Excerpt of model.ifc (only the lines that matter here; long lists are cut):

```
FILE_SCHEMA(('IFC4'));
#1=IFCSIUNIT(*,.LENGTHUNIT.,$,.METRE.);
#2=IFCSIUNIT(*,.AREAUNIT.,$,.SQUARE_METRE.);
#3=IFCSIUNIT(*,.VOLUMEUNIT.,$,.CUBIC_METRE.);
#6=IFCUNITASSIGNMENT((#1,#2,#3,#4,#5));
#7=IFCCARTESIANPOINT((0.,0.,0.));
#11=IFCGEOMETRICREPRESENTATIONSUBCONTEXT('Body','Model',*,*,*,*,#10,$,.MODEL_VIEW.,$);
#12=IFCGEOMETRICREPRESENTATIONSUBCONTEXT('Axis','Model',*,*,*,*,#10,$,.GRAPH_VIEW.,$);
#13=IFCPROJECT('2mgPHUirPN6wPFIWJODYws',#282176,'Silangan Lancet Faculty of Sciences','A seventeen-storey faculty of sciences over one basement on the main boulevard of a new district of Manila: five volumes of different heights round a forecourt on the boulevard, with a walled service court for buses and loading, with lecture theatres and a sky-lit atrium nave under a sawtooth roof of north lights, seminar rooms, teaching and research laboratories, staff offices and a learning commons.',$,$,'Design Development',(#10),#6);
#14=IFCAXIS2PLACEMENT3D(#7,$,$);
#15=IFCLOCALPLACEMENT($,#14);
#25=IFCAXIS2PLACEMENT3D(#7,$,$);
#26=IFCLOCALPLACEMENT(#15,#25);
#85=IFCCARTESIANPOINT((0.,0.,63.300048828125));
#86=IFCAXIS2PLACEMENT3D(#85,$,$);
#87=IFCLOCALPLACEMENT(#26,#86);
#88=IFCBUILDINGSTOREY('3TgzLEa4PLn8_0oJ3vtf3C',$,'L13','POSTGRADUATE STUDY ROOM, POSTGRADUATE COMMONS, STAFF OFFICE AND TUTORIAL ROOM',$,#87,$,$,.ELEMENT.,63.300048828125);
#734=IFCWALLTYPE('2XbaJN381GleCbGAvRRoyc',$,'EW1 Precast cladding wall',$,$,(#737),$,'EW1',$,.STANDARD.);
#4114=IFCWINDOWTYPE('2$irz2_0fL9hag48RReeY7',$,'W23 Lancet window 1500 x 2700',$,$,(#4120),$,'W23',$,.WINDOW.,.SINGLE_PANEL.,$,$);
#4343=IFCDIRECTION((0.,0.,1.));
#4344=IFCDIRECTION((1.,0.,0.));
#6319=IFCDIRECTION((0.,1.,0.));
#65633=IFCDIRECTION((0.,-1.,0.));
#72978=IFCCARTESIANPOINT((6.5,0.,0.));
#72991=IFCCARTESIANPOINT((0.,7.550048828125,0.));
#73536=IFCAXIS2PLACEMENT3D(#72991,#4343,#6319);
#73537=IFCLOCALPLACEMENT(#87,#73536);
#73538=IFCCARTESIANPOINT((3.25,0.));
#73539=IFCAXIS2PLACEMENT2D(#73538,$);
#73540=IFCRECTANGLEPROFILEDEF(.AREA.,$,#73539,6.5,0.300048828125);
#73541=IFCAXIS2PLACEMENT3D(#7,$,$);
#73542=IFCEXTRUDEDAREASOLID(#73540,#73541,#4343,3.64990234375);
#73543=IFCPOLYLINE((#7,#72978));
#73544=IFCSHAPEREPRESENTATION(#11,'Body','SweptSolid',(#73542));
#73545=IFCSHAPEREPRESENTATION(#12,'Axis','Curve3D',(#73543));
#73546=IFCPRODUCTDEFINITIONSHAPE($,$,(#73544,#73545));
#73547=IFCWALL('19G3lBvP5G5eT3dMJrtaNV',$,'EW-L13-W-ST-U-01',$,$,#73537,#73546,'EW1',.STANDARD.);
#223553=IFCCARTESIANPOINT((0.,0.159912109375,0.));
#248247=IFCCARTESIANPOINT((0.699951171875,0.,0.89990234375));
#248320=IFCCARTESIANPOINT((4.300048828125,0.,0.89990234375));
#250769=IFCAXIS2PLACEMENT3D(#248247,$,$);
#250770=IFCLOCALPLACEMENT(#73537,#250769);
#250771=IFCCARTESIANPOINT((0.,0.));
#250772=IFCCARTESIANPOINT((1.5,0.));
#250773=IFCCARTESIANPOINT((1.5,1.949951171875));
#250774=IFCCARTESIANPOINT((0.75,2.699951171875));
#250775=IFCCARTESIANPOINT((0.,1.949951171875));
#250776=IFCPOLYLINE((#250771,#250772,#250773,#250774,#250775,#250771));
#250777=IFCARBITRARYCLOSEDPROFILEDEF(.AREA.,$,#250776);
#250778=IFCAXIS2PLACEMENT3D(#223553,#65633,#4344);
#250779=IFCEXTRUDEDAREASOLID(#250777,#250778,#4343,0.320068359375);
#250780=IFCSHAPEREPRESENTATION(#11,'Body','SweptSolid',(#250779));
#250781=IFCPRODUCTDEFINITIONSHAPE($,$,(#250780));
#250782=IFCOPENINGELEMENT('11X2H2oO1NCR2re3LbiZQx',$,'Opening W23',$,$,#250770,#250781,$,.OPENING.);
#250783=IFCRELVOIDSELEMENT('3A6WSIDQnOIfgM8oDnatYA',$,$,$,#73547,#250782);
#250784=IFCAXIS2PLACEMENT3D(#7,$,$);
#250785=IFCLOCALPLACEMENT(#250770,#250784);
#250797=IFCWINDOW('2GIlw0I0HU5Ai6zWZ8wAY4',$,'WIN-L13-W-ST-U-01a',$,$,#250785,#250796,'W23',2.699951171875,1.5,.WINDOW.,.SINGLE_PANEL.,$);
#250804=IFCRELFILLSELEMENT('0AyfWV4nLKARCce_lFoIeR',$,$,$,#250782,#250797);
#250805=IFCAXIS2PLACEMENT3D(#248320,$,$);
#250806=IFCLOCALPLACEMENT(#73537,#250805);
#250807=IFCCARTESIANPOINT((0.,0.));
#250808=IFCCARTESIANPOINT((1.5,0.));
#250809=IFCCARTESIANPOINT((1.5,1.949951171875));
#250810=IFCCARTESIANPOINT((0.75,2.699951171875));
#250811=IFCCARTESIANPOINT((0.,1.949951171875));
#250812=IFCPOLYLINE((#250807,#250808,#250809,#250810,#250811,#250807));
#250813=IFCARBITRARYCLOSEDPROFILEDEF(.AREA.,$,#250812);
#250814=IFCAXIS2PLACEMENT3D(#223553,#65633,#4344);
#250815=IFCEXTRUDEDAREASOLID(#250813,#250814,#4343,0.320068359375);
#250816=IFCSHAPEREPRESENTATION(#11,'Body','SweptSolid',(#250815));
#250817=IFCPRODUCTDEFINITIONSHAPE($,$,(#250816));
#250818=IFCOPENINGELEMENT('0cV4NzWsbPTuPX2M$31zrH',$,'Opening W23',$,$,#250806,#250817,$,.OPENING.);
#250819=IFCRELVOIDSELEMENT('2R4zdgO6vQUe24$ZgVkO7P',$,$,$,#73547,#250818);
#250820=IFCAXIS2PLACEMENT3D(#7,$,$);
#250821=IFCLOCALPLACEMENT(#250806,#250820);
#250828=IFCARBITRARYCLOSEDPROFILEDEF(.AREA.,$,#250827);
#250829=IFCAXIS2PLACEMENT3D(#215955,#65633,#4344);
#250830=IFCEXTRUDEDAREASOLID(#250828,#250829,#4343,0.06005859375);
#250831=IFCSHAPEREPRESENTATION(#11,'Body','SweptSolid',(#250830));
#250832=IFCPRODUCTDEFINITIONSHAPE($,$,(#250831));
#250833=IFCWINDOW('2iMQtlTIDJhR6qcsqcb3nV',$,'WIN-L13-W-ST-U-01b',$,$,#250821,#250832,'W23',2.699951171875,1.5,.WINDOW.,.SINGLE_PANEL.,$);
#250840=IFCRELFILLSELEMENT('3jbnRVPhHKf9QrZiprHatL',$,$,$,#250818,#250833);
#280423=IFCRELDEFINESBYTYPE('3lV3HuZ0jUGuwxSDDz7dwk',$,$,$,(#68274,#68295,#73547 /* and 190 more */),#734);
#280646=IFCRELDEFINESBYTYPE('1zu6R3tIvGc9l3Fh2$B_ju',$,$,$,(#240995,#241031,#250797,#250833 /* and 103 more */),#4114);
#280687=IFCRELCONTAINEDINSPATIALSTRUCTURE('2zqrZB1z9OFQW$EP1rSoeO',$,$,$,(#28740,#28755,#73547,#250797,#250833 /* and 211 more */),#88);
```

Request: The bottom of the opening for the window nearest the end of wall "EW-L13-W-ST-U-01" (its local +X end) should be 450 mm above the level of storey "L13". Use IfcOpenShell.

```python
import numpy as np
import ifcopenshell
import ifcopenshell.api.geometry
import ifcopenshell.geom
import ifcopenshell.util.element
import ifcopenshell.util.placement
import ifcopenshell.util.shape
import ifcopenshell.util.unit

model = ifcopenshell.open("model.ifc")
unit_scale = ifcopenshell.util.unit.calculate_unit_scale(model)

window = model.by_id(250833)
opening = window.FillsVoids[0].RelatingOpeningElement
storey = ifcopenshell.util.element.get_container(window, ifc_class="IfcBuildingStorey")
level = ifcopenshell.util.placement.get_local_placement(storey.ObjectPlacement)[2, 3]

# The opening's origin need not be at the sill, so measure its lowest point.
shape = ifcopenshell.geom.create_shape(ifcopenshell.geom.settings(), opening)
bottom = ifcopenshell.util.shape.get_shape_bottom_elevation(shape, shape.geometry) / unit_scale
dz = level + 0.45 - bottom

shift = np.array([0.0, 0.0, dz])
# The window is placed relative to its opening, so it follows when the opening moves.
matrix = ifcopenshell.util.placement.get_local_placement(opening.ObjectPlacement)
matrix[:3, 3] += shift
ifcopenshell.api.geometry.edit_object_placement(
    model, product=opening, matrix=matrix, is_si=False, should_transform_children=True
)

print(f"moved by {dz * unit_scale:+.3f} m")

model.write("model-out.ifc")
```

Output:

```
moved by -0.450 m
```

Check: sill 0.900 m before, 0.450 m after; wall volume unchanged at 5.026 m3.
